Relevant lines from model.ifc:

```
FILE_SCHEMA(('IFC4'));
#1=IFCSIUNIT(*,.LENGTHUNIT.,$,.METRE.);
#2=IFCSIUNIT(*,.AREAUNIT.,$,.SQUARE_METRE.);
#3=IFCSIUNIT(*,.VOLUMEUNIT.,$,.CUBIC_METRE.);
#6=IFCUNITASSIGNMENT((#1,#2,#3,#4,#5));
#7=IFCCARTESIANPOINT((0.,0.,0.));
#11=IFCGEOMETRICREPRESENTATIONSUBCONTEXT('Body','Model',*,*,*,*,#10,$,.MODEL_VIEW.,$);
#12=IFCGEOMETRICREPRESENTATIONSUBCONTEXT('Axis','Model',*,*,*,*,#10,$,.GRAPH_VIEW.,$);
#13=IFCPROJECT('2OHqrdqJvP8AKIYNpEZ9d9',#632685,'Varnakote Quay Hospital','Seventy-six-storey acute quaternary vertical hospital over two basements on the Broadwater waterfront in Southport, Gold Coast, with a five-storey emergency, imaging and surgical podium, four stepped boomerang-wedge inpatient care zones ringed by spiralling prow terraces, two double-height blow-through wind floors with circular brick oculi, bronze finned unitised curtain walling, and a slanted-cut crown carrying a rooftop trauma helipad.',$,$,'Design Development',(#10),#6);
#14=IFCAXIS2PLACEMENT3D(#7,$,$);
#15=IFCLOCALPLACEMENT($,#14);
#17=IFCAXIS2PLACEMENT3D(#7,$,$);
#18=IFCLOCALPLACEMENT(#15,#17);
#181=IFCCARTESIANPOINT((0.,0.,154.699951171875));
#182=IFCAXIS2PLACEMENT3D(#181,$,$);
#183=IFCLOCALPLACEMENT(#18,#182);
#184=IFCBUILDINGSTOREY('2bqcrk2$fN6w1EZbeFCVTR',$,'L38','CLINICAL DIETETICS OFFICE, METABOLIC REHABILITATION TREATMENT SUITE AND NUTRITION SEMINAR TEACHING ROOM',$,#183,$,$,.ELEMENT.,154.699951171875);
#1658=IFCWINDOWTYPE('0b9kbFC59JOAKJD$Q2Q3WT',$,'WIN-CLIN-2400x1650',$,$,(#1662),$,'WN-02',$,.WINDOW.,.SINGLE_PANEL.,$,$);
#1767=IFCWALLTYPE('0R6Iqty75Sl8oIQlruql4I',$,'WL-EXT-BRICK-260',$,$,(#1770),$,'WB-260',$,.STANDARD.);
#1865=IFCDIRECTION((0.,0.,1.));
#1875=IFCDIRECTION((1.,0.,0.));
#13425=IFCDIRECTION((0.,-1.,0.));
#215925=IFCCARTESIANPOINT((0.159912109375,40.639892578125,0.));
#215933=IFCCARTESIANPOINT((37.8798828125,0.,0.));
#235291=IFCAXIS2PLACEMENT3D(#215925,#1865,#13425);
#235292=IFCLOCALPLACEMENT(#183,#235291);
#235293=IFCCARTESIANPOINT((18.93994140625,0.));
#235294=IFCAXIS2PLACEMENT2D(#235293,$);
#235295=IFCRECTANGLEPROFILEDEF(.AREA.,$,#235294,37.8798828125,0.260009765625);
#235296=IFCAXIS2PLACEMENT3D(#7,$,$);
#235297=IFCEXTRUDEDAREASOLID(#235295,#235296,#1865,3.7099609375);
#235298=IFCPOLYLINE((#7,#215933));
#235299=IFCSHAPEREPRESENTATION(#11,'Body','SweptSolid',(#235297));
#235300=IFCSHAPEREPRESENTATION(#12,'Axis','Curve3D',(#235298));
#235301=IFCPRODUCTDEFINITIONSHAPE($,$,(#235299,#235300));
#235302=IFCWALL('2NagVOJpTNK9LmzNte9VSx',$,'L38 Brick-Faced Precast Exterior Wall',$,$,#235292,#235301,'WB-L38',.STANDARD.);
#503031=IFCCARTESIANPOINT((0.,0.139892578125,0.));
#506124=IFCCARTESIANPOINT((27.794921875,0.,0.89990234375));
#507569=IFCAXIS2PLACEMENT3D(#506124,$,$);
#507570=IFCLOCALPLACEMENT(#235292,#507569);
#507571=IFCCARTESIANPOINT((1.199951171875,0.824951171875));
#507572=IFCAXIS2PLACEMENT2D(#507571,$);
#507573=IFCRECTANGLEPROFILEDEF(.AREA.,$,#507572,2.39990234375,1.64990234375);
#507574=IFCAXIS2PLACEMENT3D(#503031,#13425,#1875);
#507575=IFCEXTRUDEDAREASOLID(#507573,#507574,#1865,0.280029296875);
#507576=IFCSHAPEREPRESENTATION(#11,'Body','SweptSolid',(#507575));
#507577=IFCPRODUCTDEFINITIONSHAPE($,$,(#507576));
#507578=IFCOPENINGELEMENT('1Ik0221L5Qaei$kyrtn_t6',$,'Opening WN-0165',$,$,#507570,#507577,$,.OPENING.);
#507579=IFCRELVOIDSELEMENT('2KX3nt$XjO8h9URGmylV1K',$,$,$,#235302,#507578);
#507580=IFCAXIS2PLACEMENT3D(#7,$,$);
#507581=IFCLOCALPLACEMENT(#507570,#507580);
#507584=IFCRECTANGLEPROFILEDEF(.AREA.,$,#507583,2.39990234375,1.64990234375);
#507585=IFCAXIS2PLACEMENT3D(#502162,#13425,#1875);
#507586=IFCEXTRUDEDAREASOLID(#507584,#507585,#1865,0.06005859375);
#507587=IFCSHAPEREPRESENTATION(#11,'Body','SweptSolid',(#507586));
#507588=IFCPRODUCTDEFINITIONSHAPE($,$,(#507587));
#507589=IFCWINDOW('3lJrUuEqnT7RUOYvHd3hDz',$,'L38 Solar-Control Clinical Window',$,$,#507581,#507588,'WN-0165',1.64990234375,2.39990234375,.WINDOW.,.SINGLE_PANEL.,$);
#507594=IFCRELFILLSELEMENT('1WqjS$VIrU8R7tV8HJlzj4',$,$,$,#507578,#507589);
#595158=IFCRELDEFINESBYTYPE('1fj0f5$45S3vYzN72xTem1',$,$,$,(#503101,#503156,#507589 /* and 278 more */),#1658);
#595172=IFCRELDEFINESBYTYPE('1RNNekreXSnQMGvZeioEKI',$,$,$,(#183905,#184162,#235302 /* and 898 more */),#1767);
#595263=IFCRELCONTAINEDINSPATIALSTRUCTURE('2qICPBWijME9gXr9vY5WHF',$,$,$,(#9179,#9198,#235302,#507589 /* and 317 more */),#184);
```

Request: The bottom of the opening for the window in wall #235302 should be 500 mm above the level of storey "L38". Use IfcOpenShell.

```python
import numpy as np
import ifcopenshell
import ifcopenshell.api.geometry
import ifcopenshell.geom
import ifcopenshell.util.element
import ifcopenshell.util.placement
import ifcopenshell.util.shape
import ifcopenshell.util.unit

model = ifcopenshell.open("model.ifc")
unit_scale = ifcopenshell.util.unit.calculate_unit_scale(model)

window = model.by_id(507589)
opening = window.FillsVoids[0].RelatingOpeningElement
storey = ifcopenshell.util.element.get_container(window, ifc_class="IfcBuildingStorey")
level = ifcopenshell.util.placement.get_local_placement(storey.ObjectPlacement)[2, 3]

# The opening's origin need not be at the sill, so measure its lowest point.
shape = ifcopenshell.geom.create_shape(ifcopenshell.geom.settings(), opening)
bottom = ifcopenshell.util.shape.get_shape_bottom_elevation(shape, shape.geometry) / unit_scale
dz = level + 0.5 - bottom

shift = np.array([0.0, 0.0, dz])
# The window is placed relative to its opening, so it follows when the opening moves.
matrix = ifcopenshell.util.placement.get_local_placement(opening.ObjectPlacement)
matrix[:3, 3] += shift
ifcopenshell.api.geometry.edit_object_placement(
    model, product=opening, matrix=matrix, is_si=False, should_transform_children=True
)

print(f"moved by {dz * unit_scale:+.3f} m")

model.write("model-out.ifc")
```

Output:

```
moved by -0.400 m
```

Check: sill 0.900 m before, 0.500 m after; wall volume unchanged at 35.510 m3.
